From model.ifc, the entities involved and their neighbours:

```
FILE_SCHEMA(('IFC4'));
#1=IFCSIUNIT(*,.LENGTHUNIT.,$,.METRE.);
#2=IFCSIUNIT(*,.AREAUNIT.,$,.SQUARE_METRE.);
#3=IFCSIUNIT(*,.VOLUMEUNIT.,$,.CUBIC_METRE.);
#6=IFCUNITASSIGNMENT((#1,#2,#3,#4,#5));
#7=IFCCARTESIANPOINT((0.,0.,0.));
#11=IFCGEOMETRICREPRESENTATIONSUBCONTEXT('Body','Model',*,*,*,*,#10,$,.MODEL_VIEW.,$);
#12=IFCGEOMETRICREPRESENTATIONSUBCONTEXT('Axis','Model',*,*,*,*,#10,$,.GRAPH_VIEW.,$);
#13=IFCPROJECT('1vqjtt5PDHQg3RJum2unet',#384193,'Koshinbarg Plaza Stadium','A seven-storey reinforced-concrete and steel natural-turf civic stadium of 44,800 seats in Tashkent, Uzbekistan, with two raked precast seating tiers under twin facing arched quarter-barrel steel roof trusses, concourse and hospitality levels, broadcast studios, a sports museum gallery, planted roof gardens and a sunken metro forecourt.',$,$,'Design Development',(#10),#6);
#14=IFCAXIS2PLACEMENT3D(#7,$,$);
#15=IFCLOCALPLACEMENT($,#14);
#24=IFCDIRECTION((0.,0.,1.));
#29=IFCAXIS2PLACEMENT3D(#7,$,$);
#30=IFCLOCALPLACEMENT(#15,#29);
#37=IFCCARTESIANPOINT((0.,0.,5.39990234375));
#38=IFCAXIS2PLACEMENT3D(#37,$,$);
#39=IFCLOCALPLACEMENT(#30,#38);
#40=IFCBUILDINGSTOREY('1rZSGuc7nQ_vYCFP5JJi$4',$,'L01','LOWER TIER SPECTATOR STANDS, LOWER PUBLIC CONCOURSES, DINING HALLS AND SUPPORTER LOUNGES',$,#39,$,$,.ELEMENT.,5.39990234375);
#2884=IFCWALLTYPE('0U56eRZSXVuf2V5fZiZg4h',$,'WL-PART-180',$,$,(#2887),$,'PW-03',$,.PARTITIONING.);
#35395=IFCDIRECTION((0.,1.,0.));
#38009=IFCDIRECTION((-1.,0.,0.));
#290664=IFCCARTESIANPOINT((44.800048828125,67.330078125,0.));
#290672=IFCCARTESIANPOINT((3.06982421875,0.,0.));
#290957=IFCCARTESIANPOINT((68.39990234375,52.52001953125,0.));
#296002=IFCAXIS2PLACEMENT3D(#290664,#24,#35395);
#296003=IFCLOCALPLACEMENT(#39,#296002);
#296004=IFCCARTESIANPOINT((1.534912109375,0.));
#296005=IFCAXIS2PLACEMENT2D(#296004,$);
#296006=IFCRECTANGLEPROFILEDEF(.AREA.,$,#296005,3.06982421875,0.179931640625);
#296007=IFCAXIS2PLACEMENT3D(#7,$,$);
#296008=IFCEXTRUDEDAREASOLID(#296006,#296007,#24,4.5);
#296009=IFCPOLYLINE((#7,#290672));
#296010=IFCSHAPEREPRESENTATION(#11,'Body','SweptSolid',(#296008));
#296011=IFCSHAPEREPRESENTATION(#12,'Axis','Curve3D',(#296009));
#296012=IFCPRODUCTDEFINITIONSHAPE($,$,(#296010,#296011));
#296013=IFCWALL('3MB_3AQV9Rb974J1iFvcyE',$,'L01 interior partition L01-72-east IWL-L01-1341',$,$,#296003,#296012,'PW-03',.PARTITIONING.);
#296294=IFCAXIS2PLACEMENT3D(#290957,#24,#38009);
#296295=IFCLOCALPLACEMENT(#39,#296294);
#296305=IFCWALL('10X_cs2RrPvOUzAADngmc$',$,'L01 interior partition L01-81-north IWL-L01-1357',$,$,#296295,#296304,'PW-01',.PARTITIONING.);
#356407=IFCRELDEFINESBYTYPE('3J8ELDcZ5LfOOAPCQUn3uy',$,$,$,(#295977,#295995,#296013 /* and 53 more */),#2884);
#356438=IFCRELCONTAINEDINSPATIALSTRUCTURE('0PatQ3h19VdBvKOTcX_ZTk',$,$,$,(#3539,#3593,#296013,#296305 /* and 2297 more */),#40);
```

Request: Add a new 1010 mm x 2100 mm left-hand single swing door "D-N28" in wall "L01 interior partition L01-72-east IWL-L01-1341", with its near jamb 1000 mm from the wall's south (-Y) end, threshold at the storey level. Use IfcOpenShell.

```python
import numpy as np
import ifcopenshell
import ifcopenshell.api.feature
import ifcopenshell.api.geometry
import ifcopenshell.api.root
import ifcopenshell.api.spatial
import ifcopenshell.geom
import ifcopenshell.util.element
import ifcopenshell.util.placement
import ifcopenshell.util.representation
import ifcopenshell.util.shape
import ifcopenshell.util.unit

model = ifcopenshell.open("model.ifc")
unit_scale = ifcopenshell.util.unit.calculate_unit_scale(model)
settings = ifcopenshell.geom.settings()


def volume(element):
    """Net volume in cubic metres, openings subtracted."""
    shape = ifcopenshell.geom.create_shape(settings, element)
    return ifcopenshell.util.shape.get_volume(shape.geometry)


wall = model.by_id(296013)
storey = ifcopenshell.util.element.get_container(wall, ifc_class="IfcBuildingStorey")
context = ifcopenshell.util.representation.get_context(model, "Model", "Body", "MODEL_VIEW")
before = volume(wall)

width, height, from_end, sill = 1.01, 2.1, 1, 0.0  # metres

# The wall runs along its own X axis, and the end named is its -X end.
wall_shape = ifcopenshell.geom.create_shape(settings, wall)
x, y, z = ifcopenshell.util.shape.get_vertices(wall_shape.geometry).T
start = x.min() + from_end
face, thickness = float(y.min()), float(y.max() - y.min())
wall_matrix = ifcopenshell.util.placement.get_local_placement(wall.ObjectPlacement)
level = ifcopenshell.util.placement.get_local_placement(storey.ObjectPlacement)[2, 3]


def in_wall(x, y):
    """Placement at x, y metres in the wall's axes, at sill height."""
    matrix = wall_matrix.copy()
    matrix[:, 3] = wall_matrix @ np.array([x / unit_scale, y / unit_scale, 0.0, 1.0])
    matrix[2, 3] = level + sill / unit_scale
    return matrix


# Opening: a box that overshoots both wall faces by 50 mm.
opening = ifcopenshell.api.root.create_entity(model, ifc_class="IfcOpeningElement", predefined_type="OPENING")
box = ifcopenshell.api.geometry.add_wall_representation(
    model, context=context, length=width, height=height, thickness=thickness + 0.1
)
ifcopenshell.api.geometry.assign_representation(model, product=opening, representation=box)
ifcopenshell.api.geometry.edit_object_placement(model, product=opening, matrix=in_wall(start, face - 0.05), is_si=False)
ifcopenshell.api.feature.add_feature(model, feature=opening, element=wall)

door = ifcopenshell.api.root.create_entity(model, ifc_class="IfcDoor", name="D-N28", predefined_type="DOOR")
door.OverallWidth, door.OverallHeight = width / unit_scale, height / unit_scale
door.OperationType = "SINGLE_SWING_LEFT"
body = ifcopenshell.api.geometry.add_door_representation(
    model,
    context=context,
    overall_width=door.OverallWidth,
    overall_height=door.OverallHeight,
    operation_type="SINGLE_SWING_LEFT",
    lining_properties={"LiningDepth": thickness / unit_scale, "ThresholdDepth": thickness / unit_scale},
)
ifcopenshell.api.geometry.assign_representation(model, product=door, representation=body)
ifcopenshell.api.spatial.assign_container(model, products=[door], relating_structure=storey)
ifcopenshell.api.feature.add_filling(model, opening=opening, element=door)

# The lining spans the wall, so the door starts at the wall face.
ifcopenshell.api.geometry.edit_object_placement(model, product=door, matrix=in_wall(start, face), is_si=False)

after = volume(wall)

print(f"wall volume {before:.3f} -> {after:.3f} m3")

model.write("model_v2.ifc")
```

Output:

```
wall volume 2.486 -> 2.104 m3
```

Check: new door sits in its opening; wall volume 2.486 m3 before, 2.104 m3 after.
